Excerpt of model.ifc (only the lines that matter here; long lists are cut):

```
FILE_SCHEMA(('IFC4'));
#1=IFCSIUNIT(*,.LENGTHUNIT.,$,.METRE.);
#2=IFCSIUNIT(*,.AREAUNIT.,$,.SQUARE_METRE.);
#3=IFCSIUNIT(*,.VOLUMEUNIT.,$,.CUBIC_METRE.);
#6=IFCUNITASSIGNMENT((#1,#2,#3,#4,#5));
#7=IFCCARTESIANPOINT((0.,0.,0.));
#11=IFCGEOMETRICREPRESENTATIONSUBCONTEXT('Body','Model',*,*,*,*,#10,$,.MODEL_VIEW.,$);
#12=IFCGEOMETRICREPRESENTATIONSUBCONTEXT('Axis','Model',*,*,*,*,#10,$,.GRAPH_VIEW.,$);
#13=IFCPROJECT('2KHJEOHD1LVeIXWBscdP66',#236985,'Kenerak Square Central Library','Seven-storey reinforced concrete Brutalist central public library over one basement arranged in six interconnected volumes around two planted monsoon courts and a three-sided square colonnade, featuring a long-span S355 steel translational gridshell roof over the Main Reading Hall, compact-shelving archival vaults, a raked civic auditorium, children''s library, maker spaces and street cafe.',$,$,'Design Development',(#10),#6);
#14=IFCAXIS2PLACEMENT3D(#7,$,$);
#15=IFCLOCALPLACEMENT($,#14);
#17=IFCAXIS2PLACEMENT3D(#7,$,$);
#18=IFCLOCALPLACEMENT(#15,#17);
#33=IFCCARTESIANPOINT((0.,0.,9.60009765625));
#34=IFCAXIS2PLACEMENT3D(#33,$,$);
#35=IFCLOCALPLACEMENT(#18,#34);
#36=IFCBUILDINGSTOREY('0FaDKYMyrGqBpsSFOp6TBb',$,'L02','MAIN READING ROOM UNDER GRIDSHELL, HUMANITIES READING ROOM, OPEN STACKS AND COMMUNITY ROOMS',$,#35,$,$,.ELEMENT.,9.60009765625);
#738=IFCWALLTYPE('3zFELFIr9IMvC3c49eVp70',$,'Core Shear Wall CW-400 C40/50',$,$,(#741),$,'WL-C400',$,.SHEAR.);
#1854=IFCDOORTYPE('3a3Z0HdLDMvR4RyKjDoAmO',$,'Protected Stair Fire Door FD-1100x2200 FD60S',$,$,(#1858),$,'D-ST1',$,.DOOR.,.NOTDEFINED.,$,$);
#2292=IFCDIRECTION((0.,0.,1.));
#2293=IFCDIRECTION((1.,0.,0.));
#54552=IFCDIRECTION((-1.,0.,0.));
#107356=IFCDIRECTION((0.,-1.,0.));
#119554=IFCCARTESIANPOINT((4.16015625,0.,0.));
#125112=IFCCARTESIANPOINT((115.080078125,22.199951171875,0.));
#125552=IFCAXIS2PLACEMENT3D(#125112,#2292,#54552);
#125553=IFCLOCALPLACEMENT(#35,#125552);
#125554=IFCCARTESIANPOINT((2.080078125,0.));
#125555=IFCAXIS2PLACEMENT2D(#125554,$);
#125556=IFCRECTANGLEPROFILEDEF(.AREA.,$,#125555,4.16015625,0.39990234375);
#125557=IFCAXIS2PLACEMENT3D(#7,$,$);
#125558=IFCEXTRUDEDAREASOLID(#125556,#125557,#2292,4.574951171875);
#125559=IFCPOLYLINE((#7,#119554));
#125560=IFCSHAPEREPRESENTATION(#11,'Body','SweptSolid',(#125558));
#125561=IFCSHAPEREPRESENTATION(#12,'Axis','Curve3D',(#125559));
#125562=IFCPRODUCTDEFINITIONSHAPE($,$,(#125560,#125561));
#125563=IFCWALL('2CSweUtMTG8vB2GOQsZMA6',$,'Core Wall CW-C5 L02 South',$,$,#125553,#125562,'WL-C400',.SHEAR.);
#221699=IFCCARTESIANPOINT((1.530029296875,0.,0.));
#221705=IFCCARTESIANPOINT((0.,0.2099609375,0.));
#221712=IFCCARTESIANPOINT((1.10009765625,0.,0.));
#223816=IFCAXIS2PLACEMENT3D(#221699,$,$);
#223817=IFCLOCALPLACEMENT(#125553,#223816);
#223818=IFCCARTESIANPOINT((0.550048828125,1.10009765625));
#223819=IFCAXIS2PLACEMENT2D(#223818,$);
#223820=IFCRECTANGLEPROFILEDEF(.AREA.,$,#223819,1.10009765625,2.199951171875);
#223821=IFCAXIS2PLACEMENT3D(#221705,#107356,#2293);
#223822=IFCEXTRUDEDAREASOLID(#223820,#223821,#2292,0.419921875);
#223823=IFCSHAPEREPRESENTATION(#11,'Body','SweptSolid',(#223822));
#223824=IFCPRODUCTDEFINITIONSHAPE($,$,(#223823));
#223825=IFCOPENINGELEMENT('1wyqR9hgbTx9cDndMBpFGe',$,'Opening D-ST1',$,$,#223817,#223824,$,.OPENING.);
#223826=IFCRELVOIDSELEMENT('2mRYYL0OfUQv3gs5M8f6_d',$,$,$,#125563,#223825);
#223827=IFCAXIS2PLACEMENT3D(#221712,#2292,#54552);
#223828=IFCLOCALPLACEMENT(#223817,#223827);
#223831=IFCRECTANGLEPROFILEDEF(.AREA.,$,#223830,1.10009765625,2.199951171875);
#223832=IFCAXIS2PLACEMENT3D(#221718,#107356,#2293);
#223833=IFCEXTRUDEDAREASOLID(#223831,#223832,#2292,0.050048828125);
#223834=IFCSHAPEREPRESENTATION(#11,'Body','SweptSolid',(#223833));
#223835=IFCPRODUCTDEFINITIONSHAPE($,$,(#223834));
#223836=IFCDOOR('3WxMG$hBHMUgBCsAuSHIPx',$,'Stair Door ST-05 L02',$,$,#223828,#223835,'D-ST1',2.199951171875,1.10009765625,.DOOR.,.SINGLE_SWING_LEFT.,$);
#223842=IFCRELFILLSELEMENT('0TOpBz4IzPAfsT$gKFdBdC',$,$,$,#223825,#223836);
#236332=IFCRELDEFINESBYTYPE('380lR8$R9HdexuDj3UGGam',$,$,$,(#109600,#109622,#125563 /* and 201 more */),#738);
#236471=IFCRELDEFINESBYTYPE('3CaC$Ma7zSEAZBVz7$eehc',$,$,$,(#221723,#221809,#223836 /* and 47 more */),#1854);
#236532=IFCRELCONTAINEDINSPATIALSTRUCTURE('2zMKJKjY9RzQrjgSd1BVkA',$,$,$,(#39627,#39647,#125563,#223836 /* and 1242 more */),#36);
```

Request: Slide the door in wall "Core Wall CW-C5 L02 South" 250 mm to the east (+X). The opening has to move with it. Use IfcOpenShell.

```python
import ifcopenshell
import ifcopenshell.api.geometry
import ifcopenshell.util.placement

model = ifcopenshell.open("model.ifc")

door = model.by_id(223836)
opening = door.FillsVoids[0].RelatingOpeningElement
wall = opening.VoidsElements[0].RelatingBuildingElement

wall_matrix = ifcopenshell.util.placement.get_local_placement(wall.ObjectPlacement)
shift = wall_matrix[:3, 0] * -0.25
before = ifcopenshell.util.placement.get_local_placement(door.ObjectPlacement)[:3, 3].copy()

# The door is placed relative to its opening, so it follows when the opening moves.
matrix = ifcopenshell.util.placement.get_local_placement(opening.ObjectPlacement)
matrix[:3, 3] += shift
ifcopenshell.api.geometry.edit_object_placement(
    model, product=opening, matrix=matrix, is_si=False, should_transform_children=True
)

after = ifcopenshell.util.placement.get_local_placement(door.ObjectPlacement)[:3, 3]
print("door moved by", (after - before).round(3) + 0.0)

model.write("model_updated.ifc")
```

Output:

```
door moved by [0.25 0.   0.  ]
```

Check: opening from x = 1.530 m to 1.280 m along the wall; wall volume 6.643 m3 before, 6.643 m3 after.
